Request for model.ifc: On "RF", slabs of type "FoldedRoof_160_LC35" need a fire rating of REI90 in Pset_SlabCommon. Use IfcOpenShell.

First a look at what the model holds.

```python
import ifcopenshell
import ifcopenshell.util.element

model = ifcopenshell.open("model.ifc")
print(model.schema)
storey = next(s for s in model.by_type("IfcBuildingStorey") if s.Name == "RF")
slabs = [e for e in ifcopenshell.util.element.get_decomposition(storey) if e.is_a("IfcSlab")]
seen = {}
for e in slabs:
    element_type = ifcopenshell.util.element.get_type(e)
    key = (element_type.Name if element_type != e and element_type else None, ifcopenshell.util.element.get_pset(e, "Pset_SlabCommon", "FireRating"))
    seen[key] = seen.get(key, 0) + 1
for (name, value), count in sorted(seen.items(), key=str):
    print(count, "x", name, "|", value)
```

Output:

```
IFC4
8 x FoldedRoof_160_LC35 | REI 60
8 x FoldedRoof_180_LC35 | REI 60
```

```python
import ifcopenshell
import ifcopenshell.api.pset
import ifcopenshell.util.element

model = ifcopenshell.open("model.ifc")

storey = next(s for s in model.by_type("IfcBuildingStorey") if s.Name == "RF")
slabs = [e for e in ifcopenshell.util.element.get_decomposition(storey) if e.is_a("IfcSlab")]

count = 0
for e in slabs:
    element_type = ifcopenshell.util.element.get_type(e)
    if element_type in (None, e) or element_type.Name != "FoldedRoof_160_LC35":
        continue
    # add_pset returns the element's existing set when there is one.
    pset = ifcopenshell.api.pset.add_pset(model, product=e, name="Pset_SlabCommon")
    ifcopenshell.api.pset.edit_pset(model, pset=pset, properties={"FireRating": "REI90"})
    count += 1

print(count, "slabs updated")

model.write("model_edited.ifc")
```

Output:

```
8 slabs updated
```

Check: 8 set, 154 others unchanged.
